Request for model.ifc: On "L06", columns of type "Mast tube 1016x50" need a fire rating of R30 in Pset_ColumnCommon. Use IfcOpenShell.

First a look at what the model holds.

```python
import ifcopenshell
import ifcopenshell.util.element

model = ifcopenshell.open("model.ifc")
print(model.schema)
storey = next(s for s in model.by_type("IfcBuildingStorey") if s.Name == "L06")
columns = [e for e in ifcopenshell.util.element.get_decomposition(storey) if e.is_a("IfcColumn")]
seen = {}
for e in columns:
    element_type = ifcopenshell.util.element.get_type(e)
    key = (element_type.Name if element_type != e and element_type else None, ifcopenshell.util.element.get_pset(e, "Pset_ColumnCommon", "FireRating"))
    seen[key] = seen.get(key, 0) + 1
for (name, value), count in sorted(seen.items(), key=str):
    print(count, "x", name, "|", value)
```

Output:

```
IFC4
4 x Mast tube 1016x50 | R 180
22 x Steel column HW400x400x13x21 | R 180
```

```python
import ifcopenshell
import ifcopenshell.api.pset
import ifcopenshell.util.element

model = ifcopenshell.open("model.ifc")

storey = next(s for s in model.by_type("IfcBuildingStorey") if s.Name == "L06")
columns = [e for e in ifcopenshell.util.element.get_decomposition(storey) if e.is_a("IfcColumn")]

count = 0
for e in columns:
    element_type = ifcopenshell.util.element.get_type(e)
    if element_type in (None, e) or element_type.Name != "Mast tube 1016x50":
        continue
    # add_pset returns the element's existing set when there is one.
    pset = ifcopenshell.api.pset.add_pset(model, product=e, name="Pset_ColumnCommon")
    ifcopenshell.api.pset.edit_pset(model, pset=pset, properties={"FireRating": "R30"})
    count += 1

print(count, "columns updated")

model.write("model_edited.ifc")
```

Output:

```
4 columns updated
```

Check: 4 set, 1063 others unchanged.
